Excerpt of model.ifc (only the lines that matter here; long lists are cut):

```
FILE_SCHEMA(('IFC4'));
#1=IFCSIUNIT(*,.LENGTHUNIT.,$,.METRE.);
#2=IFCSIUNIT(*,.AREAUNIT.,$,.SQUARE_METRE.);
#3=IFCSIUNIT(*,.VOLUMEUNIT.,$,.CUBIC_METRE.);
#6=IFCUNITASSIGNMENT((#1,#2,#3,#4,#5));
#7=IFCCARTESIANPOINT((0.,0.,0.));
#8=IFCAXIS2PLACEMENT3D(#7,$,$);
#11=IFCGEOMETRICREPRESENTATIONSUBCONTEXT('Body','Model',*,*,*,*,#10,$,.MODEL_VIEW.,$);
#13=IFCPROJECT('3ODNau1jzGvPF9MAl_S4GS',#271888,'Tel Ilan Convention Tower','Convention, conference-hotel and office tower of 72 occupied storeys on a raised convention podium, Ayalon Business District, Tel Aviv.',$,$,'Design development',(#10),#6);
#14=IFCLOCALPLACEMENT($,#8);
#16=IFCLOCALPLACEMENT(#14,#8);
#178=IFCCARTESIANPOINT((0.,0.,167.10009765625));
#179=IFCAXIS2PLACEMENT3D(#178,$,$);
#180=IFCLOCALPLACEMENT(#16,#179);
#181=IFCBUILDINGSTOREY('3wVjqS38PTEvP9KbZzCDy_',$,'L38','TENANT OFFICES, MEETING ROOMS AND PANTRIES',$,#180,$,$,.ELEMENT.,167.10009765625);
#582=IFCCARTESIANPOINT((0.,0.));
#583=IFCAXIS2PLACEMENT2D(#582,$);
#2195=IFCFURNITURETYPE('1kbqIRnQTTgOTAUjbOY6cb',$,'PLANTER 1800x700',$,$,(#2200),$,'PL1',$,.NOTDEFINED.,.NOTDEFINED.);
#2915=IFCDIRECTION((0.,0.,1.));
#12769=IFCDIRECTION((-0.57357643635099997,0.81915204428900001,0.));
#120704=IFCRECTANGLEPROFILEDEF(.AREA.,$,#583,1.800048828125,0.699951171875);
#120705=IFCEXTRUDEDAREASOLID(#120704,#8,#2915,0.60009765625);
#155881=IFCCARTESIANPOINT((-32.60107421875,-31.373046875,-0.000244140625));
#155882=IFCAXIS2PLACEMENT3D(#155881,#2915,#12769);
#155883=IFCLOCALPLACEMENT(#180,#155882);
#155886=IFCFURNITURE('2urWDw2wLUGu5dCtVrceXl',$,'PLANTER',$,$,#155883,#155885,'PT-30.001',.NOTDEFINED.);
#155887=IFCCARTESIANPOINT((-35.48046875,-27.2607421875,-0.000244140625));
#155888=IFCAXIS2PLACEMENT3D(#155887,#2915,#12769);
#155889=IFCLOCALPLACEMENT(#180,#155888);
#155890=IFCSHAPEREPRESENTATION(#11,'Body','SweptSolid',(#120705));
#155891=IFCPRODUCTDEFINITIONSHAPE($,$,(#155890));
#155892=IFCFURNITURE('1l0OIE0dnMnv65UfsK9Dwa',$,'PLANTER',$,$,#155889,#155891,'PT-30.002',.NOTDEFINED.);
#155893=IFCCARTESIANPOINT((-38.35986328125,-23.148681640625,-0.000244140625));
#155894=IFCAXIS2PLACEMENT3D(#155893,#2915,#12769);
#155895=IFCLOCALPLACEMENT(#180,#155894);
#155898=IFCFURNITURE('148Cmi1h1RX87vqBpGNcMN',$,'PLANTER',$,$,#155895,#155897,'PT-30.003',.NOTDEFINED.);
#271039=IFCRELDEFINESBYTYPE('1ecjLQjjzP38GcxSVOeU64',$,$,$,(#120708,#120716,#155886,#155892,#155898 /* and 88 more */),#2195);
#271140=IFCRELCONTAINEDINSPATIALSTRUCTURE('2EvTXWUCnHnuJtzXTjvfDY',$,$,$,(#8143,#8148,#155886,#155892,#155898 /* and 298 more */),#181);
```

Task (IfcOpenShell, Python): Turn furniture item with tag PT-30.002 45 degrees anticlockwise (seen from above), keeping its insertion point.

```python
import ifcopenshell
import ifcopenshell.api.geometry
import ifcopenshell.util.placement

model = ifcopenshell.open("model.ifc")

item = model.by_id(155892)
matrix = ifcopenshell.util.placement.get_local_placement(item.ObjectPlacement)
matrix = matrix @ ifcopenshell.util.placement.rotation(45, "Z")
ifcopenshell.api.geometry.edit_object_placement(model, product=item, matrix=matrix, is_si=False)

print(ifcopenshell.util.placement.get_local_placement(item.ObjectPlacement).round(3) + 0.0)

model.write("model_edited.ifc")
```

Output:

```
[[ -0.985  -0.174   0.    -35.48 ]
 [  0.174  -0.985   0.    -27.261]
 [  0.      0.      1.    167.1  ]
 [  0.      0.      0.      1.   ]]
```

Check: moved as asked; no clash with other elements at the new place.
